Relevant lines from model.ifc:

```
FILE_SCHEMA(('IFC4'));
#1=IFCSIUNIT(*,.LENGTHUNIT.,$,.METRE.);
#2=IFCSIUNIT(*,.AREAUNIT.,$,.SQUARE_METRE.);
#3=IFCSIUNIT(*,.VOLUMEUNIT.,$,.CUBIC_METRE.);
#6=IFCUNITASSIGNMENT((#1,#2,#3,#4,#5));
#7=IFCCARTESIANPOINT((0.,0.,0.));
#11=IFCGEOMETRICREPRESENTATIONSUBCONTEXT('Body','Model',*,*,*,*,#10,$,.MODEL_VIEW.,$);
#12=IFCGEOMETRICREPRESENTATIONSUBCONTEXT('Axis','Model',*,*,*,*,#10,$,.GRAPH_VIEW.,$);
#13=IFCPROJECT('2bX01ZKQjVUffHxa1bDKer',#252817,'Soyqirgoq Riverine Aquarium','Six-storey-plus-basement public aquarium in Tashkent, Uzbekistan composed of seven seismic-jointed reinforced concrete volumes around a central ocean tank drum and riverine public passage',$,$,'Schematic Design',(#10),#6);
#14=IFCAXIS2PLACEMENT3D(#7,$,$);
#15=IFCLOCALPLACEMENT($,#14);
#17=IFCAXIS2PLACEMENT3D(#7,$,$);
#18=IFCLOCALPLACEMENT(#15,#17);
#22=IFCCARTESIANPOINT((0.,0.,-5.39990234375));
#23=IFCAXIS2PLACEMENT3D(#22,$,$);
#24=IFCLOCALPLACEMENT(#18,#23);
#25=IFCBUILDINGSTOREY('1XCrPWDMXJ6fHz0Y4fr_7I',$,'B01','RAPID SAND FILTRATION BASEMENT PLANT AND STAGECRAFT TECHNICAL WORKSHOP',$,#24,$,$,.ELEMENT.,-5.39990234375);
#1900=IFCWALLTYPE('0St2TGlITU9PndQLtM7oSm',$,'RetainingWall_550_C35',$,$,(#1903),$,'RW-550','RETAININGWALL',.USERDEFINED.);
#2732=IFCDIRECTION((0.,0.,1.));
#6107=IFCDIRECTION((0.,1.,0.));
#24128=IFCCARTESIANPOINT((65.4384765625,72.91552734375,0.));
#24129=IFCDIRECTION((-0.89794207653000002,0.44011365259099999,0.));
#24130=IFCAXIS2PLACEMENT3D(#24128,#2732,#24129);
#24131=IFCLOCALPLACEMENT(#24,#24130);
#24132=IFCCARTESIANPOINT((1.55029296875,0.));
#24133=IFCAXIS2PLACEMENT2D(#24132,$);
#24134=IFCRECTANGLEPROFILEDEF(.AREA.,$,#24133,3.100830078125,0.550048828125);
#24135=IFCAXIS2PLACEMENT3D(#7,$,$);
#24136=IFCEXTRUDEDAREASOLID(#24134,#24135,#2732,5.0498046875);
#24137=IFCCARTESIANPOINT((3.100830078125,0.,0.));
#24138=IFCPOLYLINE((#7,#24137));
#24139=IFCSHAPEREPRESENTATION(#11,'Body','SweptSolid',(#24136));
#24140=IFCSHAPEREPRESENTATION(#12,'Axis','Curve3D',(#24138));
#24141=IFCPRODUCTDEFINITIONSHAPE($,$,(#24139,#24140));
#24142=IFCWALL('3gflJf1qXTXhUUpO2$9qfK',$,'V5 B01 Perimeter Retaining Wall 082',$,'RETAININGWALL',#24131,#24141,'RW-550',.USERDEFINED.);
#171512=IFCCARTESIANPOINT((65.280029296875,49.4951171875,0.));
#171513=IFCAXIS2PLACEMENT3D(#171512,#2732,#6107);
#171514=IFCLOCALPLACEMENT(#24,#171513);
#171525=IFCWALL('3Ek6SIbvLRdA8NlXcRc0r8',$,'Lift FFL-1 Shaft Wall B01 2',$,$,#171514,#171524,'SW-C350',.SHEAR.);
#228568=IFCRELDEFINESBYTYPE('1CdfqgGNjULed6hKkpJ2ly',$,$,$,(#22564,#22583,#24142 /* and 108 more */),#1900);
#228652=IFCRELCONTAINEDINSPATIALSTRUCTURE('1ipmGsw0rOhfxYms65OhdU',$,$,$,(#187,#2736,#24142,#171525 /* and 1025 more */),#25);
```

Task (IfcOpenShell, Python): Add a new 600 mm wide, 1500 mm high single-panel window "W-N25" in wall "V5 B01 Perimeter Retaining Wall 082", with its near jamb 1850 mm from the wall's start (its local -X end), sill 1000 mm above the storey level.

```python
import numpy as np
import ifcopenshell
import ifcopenshell.api.feature
import ifcopenshell.api.geometry
import ifcopenshell.api.root
import ifcopenshell.api.spatial
import ifcopenshell.geom
import ifcopenshell.util.element
import ifcopenshell.util.placement
import ifcopenshell.util.representation
import ifcopenshell.util.shape
import ifcopenshell.util.unit

model = ifcopenshell.open("model.ifc")
unit_scale = ifcopenshell.util.unit.calculate_unit_scale(model)
settings = ifcopenshell.geom.settings()


def volume(element):
    """Net volume in cubic metres, openings subtracted."""
    shape = ifcopenshell.geom.create_shape(settings, element)
    return ifcopenshell.util.shape.get_volume(shape.geometry)


wall = model.by_guid("3gflJf1qXTXhUUpO2$9qfK")
storey = ifcopenshell.util.element.get_container(wall, ifc_class="IfcBuildingStorey")
context = ifcopenshell.util.representation.get_context(model, "Model", "Body", "MODEL_VIEW")
before = volume(wall)

width, height, from_end, sill = 0.6, 1.5, 1.85, 1  # metres

# The wall runs along its own X axis, and the end named is its -X end.
wall_shape = ifcopenshell.geom.create_shape(settings, wall)
x, y, z = ifcopenshell.util.shape.get_vertices(wall_shape.geometry).T
start = x.min() + from_end
face, thickness = float(y.min()), float(y.max() - y.min())
wall_matrix = ifcopenshell.util.placement.get_local_placement(wall.ObjectPlacement)
level = ifcopenshell.util.placement.get_local_placement(storey.ObjectPlacement)[2, 3]


def in_wall(x, y):
    """Placement at x, y metres in the wall's axes, at sill height."""
    matrix = wall_matrix.copy()
    matrix[:, 3] = wall_matrix @ np.array([x / unit_scale, y / unit_scale, 0.0, 1.0])
    matrix[2, 3] = level + sill / unit_scale
    return matrix


# Opening: a box that overshoots both wall faces by 50 mm.
opening = ifcopenshell.api.root.create_entity(model, ifc_class="IfcOpeningElement", predefined_type="OPENING")
box = ifcopenshell.api.geometry.add_wall_representation(
    model, context=context, length=width, height=height, thickness=thickness + 0.1
)
ifcopenshell.api.geometry.assign_representation(model, product=opening, representation=box)
ifcopenshell.api.geometry.edit_object_placement(model, product=opening, matrix=in_wall(start, face - 0.05), is_si=False)
ifcopenshell.api.feature.add_feature(model, feature=opening, element=wall)

window = ifcopenshell.api.root.create_entity(model, ifc_class="IfcWindow", name="W-N25", predefined_type="WINDOW")
window.OverallWidth, window.OverallHeight = width / unit_scale, height / unit_scale
window.PartitioningType = "SINGLE_PANEL"
body = ifcopenshell.api.geometry.add_window_representation(
    model,
    context=context,
    overall_width=window.OverallWidth,
    overall_height=window.OverallHeight,
    partition_type="SINGLE_PANEL",
)
ifcopenshell.api.geometry.assign_representation(model, product=window, representation=body)
ifcopenshell.api.spatial.assign_container(model, products=[window], relating_structure=storey)
ifcopenshell.api.feature.add_filling(model, opening=opening, element=window)

# Centre the window in the wall's thickness.
ifcopenshell.api.geometry.edit_object_placement(model, product=window, matrix=in_wall(start, face), is_si=False)
window_shape = ifcopenshell.geom.create_shape(settings, window)
depth = ifcopenshell.util.shape.get_vertices(window_shape.geometry)[:, 1]
offset = face + thickness / 2 - (depth.min() + depth.max()) / 2
ifcopenshell.api.geometry.edit_object_placement(model, product=window, matrix=in_wall(start, offset), is_si=False)

after = volume(wall)

print(f"wall volume {before:.3f} -> {after:.3f} m3")

model.write("model_rev.ifc")
```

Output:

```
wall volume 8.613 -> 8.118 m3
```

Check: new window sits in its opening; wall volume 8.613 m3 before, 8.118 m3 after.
